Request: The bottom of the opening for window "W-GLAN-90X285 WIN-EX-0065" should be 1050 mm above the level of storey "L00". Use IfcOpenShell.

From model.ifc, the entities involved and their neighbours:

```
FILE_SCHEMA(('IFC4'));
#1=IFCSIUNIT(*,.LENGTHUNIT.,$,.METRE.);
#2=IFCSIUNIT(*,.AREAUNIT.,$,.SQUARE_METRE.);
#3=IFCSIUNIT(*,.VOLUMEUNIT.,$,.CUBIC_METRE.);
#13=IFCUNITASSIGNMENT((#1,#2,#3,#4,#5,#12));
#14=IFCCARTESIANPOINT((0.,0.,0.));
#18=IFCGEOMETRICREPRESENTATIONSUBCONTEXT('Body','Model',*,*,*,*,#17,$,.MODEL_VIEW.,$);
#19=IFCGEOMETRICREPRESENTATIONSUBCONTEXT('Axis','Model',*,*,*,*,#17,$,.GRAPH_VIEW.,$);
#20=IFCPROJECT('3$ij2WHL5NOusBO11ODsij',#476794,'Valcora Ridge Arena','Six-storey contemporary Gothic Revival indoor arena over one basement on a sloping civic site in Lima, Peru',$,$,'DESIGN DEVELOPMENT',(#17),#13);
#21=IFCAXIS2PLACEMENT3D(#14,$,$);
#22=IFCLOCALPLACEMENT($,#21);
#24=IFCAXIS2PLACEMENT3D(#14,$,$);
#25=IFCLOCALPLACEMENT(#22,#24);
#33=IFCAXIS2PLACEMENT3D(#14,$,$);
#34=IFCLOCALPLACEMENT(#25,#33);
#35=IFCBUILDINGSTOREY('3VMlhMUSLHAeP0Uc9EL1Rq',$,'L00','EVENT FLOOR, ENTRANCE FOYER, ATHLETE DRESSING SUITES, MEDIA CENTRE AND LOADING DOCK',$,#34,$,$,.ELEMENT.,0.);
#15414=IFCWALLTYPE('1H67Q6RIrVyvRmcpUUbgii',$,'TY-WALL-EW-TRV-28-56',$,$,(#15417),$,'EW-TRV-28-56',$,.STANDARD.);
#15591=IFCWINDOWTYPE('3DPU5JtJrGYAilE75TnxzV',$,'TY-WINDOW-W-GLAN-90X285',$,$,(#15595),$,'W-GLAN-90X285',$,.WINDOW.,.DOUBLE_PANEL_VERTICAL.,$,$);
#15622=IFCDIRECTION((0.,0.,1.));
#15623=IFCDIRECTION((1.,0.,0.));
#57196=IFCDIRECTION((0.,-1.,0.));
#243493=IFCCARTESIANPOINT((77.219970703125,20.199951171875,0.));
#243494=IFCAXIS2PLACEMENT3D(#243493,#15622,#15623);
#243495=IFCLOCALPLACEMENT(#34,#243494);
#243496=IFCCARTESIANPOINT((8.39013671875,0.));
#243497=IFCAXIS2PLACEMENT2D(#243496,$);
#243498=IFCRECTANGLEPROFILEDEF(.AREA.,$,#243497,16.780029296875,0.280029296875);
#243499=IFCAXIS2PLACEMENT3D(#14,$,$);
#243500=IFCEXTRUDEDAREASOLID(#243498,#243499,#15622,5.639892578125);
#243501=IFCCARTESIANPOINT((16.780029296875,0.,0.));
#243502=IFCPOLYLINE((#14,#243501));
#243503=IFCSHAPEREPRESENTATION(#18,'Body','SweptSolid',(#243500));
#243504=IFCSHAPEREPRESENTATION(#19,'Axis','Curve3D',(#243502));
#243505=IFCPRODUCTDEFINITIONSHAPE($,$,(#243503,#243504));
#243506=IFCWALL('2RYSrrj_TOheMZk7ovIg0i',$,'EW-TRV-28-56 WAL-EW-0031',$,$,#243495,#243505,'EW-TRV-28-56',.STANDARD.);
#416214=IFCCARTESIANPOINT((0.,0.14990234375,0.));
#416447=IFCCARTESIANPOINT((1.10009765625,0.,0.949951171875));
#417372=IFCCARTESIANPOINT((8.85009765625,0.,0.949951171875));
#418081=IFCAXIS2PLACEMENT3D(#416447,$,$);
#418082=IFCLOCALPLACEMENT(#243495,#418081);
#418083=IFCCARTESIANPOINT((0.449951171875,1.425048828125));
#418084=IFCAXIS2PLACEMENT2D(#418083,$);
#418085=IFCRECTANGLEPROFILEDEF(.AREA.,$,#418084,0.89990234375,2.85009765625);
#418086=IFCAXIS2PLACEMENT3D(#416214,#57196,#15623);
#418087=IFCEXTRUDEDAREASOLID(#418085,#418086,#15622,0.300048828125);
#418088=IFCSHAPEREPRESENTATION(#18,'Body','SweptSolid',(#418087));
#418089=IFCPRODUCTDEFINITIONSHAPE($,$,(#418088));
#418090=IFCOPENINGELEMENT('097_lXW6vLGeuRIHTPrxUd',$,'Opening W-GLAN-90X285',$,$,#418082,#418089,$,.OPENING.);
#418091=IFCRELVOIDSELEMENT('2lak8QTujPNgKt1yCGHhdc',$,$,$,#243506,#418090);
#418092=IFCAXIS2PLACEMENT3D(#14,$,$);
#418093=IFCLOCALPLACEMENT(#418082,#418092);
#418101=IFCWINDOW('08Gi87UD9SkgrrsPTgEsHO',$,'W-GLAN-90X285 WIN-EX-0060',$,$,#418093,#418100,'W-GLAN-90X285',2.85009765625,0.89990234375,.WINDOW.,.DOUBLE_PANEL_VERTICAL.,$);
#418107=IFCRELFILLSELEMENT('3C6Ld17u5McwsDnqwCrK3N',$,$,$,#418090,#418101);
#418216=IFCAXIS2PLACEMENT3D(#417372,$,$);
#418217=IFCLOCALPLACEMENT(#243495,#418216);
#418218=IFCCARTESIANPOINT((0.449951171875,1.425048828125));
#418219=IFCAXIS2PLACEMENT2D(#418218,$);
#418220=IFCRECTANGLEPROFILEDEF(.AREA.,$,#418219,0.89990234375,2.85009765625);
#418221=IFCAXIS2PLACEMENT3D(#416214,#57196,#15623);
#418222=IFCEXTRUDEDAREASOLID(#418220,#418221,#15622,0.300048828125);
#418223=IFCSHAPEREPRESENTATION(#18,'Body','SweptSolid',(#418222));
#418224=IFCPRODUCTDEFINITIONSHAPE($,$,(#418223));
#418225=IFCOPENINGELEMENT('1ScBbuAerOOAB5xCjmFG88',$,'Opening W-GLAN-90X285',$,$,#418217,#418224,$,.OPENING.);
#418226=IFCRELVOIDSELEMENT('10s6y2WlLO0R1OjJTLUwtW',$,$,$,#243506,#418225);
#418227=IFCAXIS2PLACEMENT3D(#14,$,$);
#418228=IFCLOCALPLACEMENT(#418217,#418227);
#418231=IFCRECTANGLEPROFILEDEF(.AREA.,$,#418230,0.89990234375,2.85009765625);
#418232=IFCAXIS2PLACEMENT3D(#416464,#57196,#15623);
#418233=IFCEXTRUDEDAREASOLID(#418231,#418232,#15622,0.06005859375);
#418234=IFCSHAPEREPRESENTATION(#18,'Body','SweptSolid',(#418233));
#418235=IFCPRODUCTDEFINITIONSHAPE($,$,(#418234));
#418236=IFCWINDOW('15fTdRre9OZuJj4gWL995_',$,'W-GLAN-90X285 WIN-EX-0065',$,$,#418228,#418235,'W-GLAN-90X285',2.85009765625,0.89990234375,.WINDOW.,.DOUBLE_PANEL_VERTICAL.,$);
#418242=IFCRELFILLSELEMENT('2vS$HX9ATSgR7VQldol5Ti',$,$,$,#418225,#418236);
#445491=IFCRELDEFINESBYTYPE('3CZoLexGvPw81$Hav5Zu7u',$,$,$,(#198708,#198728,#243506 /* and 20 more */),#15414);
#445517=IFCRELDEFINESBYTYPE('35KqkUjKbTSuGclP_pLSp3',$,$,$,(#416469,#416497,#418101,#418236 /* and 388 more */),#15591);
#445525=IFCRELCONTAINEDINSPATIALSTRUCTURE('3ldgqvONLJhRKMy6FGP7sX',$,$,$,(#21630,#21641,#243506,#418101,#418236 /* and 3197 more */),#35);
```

```python
import numpy as np
import ifcopenshell
import ifcopenshell.api.geometry
import ifcopenshell.geom
import ifcopenshell.util.element
import ifcopenshell.util.placement
import ifcopenshell.util.shape
import ifcopenshell.util.unit

model = ifcopenshell.open("model.ifc")
unit_scale = ifcopenshell.util.unit.calculate_unit_scale(model)

window = model.by_id(418236)
opening = window.FillsVoids[0].RelatingOpeningElement
storey = ifcopenshell.util.element.get_container(window, ifc_class="IfcBuildingStorey")
level = ifcopenshell.util.placement.get_local_placement(storey.ObjectPlacement)[2, 3]

# The opening's origin need not be at the sill, so measure its lowest point.
shape = ifcopenshell.geom.create_shape(ifcopenshell.geom.settings(), opening)
bottom = ifcopenshell.util.shape.get_shape_bottom_elevation(shape, shape.geometry) / unit_scale
dz = level + 1.05 / unit_scale - bottom

shift = np.array([0.0, 0.0, dz])
# The window is placed relative to its opening, so it follows when the opening moves.
matrix = ifcopenshell.util.placement.get_local_placement(opening.ObjectPlacement)
matrix[:3, 3] += shift
ifcopenshell.api.geometry.edit_object_placement(
    model, product=opening, matrix=matrix, is_si=False, should_transform_children=True
)

print(f"moved by {dz * unit_scale:+.3f} m")

model.write("model_v2.ifc")
```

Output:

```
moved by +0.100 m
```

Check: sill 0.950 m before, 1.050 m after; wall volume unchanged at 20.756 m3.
